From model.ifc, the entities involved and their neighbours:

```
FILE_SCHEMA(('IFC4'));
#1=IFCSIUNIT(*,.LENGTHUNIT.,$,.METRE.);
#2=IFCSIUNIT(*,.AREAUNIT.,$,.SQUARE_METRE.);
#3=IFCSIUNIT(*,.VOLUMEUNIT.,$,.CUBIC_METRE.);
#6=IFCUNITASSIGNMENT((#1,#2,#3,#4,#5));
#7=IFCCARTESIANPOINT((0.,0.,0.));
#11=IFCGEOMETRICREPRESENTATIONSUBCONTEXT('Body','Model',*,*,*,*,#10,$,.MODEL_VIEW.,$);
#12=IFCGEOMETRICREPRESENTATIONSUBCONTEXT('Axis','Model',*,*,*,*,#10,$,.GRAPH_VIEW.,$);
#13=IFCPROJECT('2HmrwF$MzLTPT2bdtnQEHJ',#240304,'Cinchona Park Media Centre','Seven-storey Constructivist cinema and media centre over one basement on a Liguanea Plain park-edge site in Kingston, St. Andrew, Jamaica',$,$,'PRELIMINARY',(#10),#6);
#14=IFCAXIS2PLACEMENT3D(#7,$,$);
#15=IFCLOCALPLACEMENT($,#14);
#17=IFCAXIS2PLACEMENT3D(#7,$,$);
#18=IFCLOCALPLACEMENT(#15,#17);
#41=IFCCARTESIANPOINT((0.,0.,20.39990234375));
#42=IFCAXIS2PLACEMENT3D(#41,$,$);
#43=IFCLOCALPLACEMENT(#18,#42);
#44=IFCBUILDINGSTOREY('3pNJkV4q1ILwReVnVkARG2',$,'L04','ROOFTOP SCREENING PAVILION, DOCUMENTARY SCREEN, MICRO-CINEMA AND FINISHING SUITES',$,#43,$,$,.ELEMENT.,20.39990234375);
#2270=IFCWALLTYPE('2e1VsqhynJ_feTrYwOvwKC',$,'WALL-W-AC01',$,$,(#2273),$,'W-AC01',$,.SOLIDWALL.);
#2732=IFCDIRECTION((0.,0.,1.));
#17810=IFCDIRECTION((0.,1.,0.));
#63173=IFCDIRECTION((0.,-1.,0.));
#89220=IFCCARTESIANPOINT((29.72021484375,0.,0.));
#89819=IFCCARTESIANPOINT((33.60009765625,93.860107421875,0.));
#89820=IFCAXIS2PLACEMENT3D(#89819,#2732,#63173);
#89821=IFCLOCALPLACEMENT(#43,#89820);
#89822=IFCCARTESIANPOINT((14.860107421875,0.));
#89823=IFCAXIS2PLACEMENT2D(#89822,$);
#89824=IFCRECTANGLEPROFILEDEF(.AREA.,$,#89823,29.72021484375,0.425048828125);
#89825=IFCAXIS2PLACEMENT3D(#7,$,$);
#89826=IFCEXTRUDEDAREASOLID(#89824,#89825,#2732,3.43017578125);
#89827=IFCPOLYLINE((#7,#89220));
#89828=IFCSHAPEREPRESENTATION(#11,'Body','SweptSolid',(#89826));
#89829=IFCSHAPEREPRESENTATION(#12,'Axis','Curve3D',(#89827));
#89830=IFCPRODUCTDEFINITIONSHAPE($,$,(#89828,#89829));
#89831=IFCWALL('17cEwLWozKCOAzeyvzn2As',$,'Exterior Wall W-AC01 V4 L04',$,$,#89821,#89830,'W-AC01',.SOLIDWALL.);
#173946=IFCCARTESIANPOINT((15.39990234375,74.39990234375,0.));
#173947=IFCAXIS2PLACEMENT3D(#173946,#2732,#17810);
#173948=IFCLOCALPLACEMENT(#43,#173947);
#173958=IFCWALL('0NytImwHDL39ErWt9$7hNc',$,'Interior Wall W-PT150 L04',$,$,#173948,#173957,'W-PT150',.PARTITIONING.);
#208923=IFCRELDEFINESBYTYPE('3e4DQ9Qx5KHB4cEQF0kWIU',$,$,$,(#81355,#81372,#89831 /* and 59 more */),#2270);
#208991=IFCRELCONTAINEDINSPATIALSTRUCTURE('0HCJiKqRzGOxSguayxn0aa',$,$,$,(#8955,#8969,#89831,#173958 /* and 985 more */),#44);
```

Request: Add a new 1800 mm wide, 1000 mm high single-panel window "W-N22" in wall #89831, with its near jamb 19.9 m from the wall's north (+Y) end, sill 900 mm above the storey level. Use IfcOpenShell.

```python
import numpy as np
import ifcopenshell
import ifcopenshell.api.feature
import ifcopenshell.api.geometry
import ifcopenshell.api.root
import ifcopenshell.api.spatial
import ifcopenshell.geom
import ifcopenshell.util.element
import ifcopenshell.util.placement
import ifcopenshell.util.representation
import ifcopenshell.util.shape
import ifcopenshell.util.unit

model = ifcopenshell.open("model.ifc")
unit_scale = ifcopenshell.util.unit.calculate_unit_scale(model)
settings = ifcopenshell.geom.settings()


def volume(element):
    """Net volume in cubic metres, openings subtracted."""
    shape = ifcopenshell.geom.create_shape(settings, element)
    return ifcopenshell.util.shape.get_volume(shape.geometry)


wall = model.by_id(89831)
storey = ifcopenshell.util.element.get_container(wall, ifc_class="IfcBuildingStorey")
context = ifcopenshell.util.representation.get_context(model, "Model", "Body", "MODEL_VIEW")
before = volume(wall)

width, height, from_end, sill = 1.8, 1, 19.9, 0.9  # metres

# The wall runs along its own X axis, and the end named is its -X end.
wall_shape = ifcopenshell.geom.create_shape(settings, wall)
x, y, z = ifcopenshell.util.shape.get_vertices(wall_shape.geometry).T
start = x.min() + from_end
face, thickness = float(y.min()), float(y.max() - y.min())
wall_matrix = ifcopenshell.util.placement.get_local_placement(wall.ObjectPlacement)
level = ifcopenshell.util.placement.get_local_placement(storey.ObjectPlacement)[2, 3]


def in_wall(x, y):
    """Placement at x, y metres in the wall's axes, at sill height."""
    matrix = wall_matrix.copy()
    matrix[:, 3] = wall_matrix @ np.array([x / unit_scale, y / unit_scale, 0.0, 1.0])
    matrix[2, 3] = level + sill / unit_scale
    return matrix


# Opening: a box that overshoots both wall faces by 50 mm.
opening = ifcopenshell.api.root.create_entity(model, ifc_class="IfcOpeningElement", predefined_type="OPENING")
box = ifcopenshell.api.geometry.add_wall_representation(
    model, context=context, length=width, height=height, thickness=thickness + 0.1
)
ifcopenshell.api.geometry.assign_representation(model, product=opening, representation=box)
ifcopenshell.api.geometry.edit_object_placement(model, product=opening, matrix=in_wall(start, face - 0.05), is_si=False)
ifcopenshell.api.feature.add_feature(model, feature=opening, element=wall)

window = ifcopenshell.api.root.create_entity(model, ifc_class="IfcWindow", name="W-N22", predefined_type="WINDOW")
window.OverallWidth, window.OverallHeight = width / unit_scale, height / unit_scale
window.PartitioningType = "SINGLE_PANEL"
body = ifcopenshell.api.geometry.add_window_representation(
    model,
    context=context,
    overall_width=window.OverallWidth,
    overall_height=window.OverallHeight,
    partition_type="SINGLE_PANEL",
)
ifcopenshell.api.geometry.assign_representation(model, product=window, representation=body)
ifcopenshell.api.spatial.assign_container(model, products=[window], relating_structure=storey)
ifcopenshell.api.feature.add_filling(model, opening=opening, element=window)

# Centre the window in the wall's thickness.
ifcopenshell.api.geometry.edit_object_placement(model, product=window, matrix=in_wall(start, face), is_si=False)
window_shape = ifcopenshell.geom.create_shape(settings, window)
depth = ifcopenshell.util.shape.get_vertices(window_shape.geometry)[:, 1]
offset = face + thickness / 2 - (depth.min() + depth.max()) / 2
ifcopenshell.api.geometry.edit_object_placement(model, product=window, matrix=in_wall(start, offset), is_si=False)

after = volume(wall)

print(f"wall volume {before:.3f} -> {after:.3f} m3")

model.write("model_v2.ifc")
```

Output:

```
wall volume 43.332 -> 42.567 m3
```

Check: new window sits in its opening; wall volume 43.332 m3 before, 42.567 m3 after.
